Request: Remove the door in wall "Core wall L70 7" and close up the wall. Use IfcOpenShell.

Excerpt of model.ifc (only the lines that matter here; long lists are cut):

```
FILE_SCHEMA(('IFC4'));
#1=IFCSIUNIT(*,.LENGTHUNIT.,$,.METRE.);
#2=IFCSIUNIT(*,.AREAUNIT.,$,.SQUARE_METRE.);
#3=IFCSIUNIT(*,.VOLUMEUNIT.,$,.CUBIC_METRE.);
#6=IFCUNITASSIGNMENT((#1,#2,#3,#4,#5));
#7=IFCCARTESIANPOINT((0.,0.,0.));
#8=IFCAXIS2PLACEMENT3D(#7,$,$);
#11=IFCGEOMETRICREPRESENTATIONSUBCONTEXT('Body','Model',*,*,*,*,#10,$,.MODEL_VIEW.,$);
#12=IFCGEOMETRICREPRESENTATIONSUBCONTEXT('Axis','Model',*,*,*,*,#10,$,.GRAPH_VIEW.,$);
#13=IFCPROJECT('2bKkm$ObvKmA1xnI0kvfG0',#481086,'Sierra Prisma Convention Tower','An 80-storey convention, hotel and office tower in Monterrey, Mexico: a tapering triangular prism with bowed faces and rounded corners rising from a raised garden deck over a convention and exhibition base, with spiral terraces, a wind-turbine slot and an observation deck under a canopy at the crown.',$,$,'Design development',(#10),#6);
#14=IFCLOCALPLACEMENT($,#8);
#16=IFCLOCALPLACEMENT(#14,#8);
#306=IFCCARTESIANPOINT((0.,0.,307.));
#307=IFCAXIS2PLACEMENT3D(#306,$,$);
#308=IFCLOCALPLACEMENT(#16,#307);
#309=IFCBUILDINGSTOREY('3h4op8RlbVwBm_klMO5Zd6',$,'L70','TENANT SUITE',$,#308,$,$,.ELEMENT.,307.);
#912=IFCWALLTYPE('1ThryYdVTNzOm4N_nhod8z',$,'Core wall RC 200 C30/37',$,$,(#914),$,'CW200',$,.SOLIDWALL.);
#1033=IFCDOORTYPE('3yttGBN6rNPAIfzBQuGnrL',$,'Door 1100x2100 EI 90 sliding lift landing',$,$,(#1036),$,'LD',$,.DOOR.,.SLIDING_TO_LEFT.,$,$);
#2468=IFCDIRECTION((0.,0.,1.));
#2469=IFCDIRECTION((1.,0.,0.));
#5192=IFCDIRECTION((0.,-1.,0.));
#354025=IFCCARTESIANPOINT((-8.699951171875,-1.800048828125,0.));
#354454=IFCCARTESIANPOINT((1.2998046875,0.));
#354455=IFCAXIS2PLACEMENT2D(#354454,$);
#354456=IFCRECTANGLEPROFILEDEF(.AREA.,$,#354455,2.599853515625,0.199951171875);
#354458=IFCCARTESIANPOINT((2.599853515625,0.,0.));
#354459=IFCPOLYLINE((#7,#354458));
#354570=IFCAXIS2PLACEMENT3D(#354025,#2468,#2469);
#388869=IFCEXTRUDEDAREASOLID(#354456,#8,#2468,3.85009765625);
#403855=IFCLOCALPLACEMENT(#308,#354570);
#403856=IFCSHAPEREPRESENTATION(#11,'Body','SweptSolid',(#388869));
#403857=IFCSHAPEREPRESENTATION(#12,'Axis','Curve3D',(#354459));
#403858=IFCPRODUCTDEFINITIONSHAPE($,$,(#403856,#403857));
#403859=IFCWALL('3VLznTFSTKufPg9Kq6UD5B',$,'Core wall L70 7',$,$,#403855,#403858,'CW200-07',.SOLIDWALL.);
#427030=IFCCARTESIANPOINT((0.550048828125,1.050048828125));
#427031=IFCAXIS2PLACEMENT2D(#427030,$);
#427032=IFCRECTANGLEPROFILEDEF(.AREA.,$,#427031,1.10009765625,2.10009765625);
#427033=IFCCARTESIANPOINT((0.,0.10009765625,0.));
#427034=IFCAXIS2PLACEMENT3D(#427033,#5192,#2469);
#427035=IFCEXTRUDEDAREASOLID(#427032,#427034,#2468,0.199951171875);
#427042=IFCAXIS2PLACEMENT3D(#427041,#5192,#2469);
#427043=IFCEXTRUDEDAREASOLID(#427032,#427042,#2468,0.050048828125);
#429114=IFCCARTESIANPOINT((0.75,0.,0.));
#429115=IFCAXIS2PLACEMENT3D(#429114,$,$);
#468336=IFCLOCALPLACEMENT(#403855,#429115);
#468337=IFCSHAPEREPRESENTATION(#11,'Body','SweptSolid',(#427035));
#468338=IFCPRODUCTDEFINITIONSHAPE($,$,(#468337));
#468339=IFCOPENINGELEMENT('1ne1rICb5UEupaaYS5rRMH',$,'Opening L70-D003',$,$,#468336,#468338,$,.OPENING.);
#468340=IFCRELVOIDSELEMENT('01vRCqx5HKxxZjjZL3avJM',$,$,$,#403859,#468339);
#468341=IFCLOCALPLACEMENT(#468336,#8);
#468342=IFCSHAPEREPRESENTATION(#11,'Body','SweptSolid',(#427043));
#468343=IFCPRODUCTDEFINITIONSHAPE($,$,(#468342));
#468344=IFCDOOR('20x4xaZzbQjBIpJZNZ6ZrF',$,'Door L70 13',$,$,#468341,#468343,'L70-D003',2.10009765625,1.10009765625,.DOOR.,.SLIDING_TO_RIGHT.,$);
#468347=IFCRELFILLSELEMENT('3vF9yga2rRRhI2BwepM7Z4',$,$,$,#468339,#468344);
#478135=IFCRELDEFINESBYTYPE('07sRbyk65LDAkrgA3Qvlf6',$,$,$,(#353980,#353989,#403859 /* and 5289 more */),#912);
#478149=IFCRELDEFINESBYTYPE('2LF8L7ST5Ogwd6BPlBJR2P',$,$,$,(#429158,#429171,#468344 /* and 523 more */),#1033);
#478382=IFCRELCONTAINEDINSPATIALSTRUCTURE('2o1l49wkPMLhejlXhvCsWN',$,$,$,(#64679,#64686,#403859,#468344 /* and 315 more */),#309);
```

```python
import ifcopenshell
import ifcopenshell.api.feature
import ifcopenshell.api.root
import ifcopenshell.geom
import ifcopenshell.util.shape

model = ifcopenshell.open("model.ifc")
settings = ifcopenshell.geom.settings()


def volume(element):
    """Net volume in cubic metres, openings subtracted."""
    shape = ifcopenshell.geom.create_shape(settings, element)
    return ifcopenshell.util.shape.get_volume(shape.geometry)


door = model.by_guid("20x4xaZzbQjBIpJZNZ6ZrF")
opening = door.FillsVoids[0].RelatingOpeningElement
wall = opening.VoidsElements[0].RelatingBuildingElement
before = volume(wall)

ifcopenshell.api.root.remove_product(model, product=door)
ifcopenshell.api.feature.remove_feature(model, feature=opening)

after = volume(wall)

print(f"wall volume {before:.3f} -> {after:.3f} m3")

model.write("model-out.ifc")
```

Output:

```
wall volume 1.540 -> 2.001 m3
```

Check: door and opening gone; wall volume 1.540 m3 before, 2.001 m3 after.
